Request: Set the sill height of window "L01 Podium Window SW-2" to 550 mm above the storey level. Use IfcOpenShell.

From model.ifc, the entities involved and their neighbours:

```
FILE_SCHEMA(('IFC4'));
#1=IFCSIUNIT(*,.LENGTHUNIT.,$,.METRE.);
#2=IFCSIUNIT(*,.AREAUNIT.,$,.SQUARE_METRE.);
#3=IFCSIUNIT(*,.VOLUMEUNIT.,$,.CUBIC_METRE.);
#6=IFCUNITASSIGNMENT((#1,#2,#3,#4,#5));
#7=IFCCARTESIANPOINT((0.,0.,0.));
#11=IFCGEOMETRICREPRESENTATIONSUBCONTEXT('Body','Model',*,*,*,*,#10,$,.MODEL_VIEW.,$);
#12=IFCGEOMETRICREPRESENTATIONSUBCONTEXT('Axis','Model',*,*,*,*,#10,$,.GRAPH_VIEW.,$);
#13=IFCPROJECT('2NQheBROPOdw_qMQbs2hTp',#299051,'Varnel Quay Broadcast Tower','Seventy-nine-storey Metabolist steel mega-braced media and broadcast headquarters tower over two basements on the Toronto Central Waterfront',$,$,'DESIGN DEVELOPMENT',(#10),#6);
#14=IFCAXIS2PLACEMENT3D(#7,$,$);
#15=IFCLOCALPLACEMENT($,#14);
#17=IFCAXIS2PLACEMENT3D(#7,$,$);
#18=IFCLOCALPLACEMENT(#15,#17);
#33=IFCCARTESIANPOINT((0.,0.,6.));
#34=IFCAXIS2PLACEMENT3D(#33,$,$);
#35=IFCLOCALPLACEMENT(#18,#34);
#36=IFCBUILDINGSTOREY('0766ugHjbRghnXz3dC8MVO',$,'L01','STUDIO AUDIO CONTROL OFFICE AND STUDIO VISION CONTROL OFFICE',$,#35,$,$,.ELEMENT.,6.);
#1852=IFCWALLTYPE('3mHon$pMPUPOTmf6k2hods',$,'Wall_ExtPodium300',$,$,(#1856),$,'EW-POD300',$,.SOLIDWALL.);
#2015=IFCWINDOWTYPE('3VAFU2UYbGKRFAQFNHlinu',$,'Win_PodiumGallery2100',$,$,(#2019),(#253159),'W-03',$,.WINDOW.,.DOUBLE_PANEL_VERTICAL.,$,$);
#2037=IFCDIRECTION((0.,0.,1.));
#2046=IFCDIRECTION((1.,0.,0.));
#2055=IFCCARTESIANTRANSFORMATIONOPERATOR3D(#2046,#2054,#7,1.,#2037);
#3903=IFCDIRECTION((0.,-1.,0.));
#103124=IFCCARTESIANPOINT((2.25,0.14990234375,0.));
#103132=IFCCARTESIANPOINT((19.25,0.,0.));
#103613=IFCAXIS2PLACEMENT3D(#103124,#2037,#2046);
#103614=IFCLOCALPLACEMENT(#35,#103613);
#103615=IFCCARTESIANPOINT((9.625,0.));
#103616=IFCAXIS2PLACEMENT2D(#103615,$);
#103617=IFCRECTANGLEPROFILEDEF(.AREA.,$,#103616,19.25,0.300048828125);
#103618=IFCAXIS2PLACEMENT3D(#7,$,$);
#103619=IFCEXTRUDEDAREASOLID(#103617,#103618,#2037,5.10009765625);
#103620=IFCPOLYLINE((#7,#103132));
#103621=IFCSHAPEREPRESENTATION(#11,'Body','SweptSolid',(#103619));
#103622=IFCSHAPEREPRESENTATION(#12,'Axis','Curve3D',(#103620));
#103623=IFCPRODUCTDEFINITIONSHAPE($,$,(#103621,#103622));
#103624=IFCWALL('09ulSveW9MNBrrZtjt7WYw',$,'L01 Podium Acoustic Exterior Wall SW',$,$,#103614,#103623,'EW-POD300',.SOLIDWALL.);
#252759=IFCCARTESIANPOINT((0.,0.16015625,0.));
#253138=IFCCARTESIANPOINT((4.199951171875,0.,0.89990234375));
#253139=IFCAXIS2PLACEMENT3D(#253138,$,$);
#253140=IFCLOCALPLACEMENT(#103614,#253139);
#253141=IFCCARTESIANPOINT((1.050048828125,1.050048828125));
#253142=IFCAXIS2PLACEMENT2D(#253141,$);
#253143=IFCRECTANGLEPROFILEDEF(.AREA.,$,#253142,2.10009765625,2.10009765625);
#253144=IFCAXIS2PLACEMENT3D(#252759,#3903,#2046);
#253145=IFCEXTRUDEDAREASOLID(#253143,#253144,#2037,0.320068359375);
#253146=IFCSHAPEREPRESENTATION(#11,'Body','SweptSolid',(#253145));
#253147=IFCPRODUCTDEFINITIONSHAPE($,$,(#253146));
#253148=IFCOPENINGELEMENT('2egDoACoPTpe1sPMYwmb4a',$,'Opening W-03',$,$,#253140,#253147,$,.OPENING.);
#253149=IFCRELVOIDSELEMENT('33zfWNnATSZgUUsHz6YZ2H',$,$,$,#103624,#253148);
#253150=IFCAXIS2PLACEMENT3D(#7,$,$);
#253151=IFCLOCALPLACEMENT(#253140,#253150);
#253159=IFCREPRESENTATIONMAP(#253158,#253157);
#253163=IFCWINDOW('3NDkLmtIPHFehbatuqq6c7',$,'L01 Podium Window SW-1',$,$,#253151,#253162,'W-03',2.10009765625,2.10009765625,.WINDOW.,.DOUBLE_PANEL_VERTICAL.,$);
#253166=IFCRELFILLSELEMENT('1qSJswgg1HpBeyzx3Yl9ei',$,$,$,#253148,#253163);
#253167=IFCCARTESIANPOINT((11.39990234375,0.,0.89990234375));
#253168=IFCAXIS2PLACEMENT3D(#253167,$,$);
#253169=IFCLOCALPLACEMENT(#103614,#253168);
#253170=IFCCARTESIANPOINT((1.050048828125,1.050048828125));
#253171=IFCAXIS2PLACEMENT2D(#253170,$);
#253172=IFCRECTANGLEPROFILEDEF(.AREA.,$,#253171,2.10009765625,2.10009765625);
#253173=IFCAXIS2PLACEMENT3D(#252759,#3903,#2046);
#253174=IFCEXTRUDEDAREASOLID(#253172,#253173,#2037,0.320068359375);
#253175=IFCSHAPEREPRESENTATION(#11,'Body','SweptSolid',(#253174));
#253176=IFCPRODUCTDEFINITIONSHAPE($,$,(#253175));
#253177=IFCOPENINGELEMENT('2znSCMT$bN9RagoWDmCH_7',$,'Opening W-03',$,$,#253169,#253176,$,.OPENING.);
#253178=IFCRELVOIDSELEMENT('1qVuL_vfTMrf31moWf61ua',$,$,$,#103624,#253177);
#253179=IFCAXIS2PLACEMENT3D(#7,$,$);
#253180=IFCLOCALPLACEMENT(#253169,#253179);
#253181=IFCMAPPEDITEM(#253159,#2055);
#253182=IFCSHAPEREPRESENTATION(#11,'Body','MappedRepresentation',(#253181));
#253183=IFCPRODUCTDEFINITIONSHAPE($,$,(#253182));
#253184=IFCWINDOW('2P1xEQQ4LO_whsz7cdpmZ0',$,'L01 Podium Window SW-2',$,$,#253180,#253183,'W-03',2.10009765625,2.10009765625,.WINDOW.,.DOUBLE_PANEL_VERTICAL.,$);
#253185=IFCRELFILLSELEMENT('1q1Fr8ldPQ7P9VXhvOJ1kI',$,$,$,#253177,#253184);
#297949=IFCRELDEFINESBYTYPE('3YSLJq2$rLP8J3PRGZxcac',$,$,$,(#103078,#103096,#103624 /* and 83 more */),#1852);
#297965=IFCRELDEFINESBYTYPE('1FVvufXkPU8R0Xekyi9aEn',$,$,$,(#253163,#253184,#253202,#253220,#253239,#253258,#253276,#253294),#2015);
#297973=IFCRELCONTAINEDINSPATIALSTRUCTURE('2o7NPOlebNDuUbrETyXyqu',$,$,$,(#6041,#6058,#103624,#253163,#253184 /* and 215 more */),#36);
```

```python
import numpy as np
import ifcopenshell
import ifcopenshell.api.geometry
import ifcopenshell.geom
import ifcopenshell.util.element
import ifcopenshell.util.placement
import ifcopenshell.util.shape
import ifcopenshell.util.unit

model = ifcopenshell.open("model.ifc")
unit_scale = ifcopenshell.util.unit.calculate_unit_scale(model)

window = model.by_id(253184)
opening = window.FillsVoids[0].RelatingOpeningElement
storey = ifcopenshell.util.element.get_container(window, ifc_class="IfcBuildingStorey")
level = ifcopenshell.util.placement.get_local_placement(storey.ObjectPlacement)[2, 3]

# The opening's origin need not be at the sill, so measure its lowest point.
shape = ifcopenshell.geom.create_shape(ifcopenshell.geom.settings(), opening)
bottom = ifcopenshell.util.shape.get_shape_bottom_elevation(shape, shape.geometry) / unit_scale
dz = level + 0.55 / unit_scale - bottom

shift = np.array([0.0, 0.0, dz])
# The window is placed relative to its opening, so it follows when the opening moves.
matrix = ifcopenshell.util.placement.get_local_placement(opening.ObjectPlacement)
matrix[:3, 3] += shift
ifcopenshell.api.geometry.edit_object_placement(
    model, product=opening, matrix=matrix, is_si=False, should_transform_children=True
)

print(f"moved by {dz * unit_scale:+.3f} m")

model.write("model_rev.ifc")
```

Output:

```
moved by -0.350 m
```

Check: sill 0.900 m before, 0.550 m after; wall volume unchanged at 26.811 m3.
